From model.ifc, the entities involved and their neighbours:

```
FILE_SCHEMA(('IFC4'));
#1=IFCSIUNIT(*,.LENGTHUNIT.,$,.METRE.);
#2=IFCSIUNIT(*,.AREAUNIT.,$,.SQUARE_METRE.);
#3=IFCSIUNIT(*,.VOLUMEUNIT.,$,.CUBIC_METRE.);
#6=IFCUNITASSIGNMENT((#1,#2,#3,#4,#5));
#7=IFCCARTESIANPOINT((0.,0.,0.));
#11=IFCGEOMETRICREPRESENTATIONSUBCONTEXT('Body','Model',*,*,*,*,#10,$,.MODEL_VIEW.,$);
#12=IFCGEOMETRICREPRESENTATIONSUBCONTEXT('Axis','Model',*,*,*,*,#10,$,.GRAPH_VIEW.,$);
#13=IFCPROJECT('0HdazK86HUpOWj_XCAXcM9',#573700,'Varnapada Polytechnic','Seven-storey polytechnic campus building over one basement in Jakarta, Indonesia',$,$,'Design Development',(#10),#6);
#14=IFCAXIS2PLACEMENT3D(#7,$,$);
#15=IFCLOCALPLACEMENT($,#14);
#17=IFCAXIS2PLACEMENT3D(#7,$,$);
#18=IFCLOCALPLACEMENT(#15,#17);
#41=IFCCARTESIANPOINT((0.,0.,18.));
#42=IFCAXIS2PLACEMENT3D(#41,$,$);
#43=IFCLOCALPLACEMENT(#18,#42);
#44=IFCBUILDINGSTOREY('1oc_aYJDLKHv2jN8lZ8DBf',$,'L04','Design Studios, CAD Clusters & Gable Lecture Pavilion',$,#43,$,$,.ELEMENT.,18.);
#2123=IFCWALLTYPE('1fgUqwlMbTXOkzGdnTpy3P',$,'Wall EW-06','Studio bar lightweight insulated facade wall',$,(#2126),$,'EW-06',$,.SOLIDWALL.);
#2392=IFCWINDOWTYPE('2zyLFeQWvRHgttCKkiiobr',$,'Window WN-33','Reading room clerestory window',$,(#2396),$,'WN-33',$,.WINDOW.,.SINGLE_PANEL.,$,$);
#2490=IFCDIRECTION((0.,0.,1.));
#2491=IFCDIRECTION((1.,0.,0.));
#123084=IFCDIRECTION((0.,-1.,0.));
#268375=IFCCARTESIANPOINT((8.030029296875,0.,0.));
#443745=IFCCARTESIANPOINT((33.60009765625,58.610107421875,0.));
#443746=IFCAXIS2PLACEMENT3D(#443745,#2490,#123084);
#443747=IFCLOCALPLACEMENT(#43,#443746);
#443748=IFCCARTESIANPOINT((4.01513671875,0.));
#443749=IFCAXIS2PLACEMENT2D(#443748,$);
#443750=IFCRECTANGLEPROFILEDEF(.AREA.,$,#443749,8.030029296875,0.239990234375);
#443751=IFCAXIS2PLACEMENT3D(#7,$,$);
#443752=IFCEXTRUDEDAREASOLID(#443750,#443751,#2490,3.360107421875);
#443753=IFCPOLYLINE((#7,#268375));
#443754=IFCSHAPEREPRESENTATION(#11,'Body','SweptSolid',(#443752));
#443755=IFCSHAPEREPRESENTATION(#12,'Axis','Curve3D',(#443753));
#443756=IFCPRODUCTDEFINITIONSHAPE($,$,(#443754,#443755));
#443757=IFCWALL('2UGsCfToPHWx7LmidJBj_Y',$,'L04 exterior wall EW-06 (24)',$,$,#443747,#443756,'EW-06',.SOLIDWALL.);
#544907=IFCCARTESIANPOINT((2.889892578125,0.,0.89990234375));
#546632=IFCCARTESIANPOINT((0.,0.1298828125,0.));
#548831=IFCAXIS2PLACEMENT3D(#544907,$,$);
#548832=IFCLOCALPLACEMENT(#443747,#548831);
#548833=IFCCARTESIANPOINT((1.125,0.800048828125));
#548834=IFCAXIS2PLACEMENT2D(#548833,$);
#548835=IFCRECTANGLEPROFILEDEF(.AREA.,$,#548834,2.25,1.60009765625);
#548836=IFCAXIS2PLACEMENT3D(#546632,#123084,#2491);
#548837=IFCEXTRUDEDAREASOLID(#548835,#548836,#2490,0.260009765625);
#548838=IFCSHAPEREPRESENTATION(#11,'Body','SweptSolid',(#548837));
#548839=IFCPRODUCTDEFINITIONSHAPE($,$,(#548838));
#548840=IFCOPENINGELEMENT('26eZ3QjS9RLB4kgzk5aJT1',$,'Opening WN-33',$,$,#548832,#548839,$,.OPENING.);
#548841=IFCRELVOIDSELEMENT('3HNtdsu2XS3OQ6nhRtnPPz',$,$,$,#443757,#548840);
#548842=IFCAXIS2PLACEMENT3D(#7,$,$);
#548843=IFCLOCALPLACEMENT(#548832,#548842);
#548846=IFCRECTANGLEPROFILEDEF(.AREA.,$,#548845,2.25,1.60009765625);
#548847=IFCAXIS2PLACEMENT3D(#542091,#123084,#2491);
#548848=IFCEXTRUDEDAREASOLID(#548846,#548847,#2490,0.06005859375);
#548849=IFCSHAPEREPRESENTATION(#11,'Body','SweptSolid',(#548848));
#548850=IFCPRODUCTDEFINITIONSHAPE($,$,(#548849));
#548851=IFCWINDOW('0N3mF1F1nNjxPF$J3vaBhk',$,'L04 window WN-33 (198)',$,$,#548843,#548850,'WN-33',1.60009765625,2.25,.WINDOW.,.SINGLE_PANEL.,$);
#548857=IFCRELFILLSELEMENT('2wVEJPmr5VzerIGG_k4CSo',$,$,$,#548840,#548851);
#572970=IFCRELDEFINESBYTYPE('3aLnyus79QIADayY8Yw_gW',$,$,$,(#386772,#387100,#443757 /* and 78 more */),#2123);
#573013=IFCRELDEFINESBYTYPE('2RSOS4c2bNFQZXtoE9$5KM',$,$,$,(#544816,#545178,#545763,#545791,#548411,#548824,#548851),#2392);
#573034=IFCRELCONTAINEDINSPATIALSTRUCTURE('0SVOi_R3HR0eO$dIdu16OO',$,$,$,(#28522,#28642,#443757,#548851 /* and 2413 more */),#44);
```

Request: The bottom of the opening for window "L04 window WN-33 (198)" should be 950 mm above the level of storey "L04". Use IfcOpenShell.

```python
import numpy as np
import ifcopenshell
import ifcopenshell.api.geometry
import ifcopenshell.geom
import ifcopenshell.util.element
import ifcopenshell.util.placement
import ifcopenshell.util.shape
import ifcopenshell.util.unit

model = ifcopenshell.open("model.ifc")
unit_scale = ifcopenshell.util.unit.calculate_unit_scale(model)

window = model.by_guid("0N3mF1F1nNjxPF$J3vaBhk")
opening = window.FillsVoids[0].RelatingOpeningElement
storey = ifcopenshell.util.element.get_container(window, ifc_class="IfcBuildingStorey")
level = ifcopenshell.util.placement.get_local_placement(storey.ObjectPlacement)[2, 3]

# The opening's origin need not be at the sill, so measure its lowest point.
shape = ifcopenshell.geom.create_shape(ifcopenshell.geom.settings(), opening)
bottom = ifcopenshell.util.shape.get_shape_bottom_elevation(shape, shape.geometry) / unit_scale
dz = level + 0.95 / unit_scale - bottom

shift = np.array([0.0, 0.0, dz])
# The window is placed relative to its opening, so it follows when the opening moves.
matrix = ifcopenshell.util.placement.get_local_placement(opening.ObjectPlacement)
matrix[:3, 3] += shift
ifcopenshell.api.geometry.edit_object_placement(
    model, product=opening, matrix=matrix, is_si=False, should_transform_children=True
)

print(f"moved by {dz * unit_scale:+.3f} m")

model.write("model_rev.ifc")
```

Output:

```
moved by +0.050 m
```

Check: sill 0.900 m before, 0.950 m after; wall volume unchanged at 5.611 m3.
